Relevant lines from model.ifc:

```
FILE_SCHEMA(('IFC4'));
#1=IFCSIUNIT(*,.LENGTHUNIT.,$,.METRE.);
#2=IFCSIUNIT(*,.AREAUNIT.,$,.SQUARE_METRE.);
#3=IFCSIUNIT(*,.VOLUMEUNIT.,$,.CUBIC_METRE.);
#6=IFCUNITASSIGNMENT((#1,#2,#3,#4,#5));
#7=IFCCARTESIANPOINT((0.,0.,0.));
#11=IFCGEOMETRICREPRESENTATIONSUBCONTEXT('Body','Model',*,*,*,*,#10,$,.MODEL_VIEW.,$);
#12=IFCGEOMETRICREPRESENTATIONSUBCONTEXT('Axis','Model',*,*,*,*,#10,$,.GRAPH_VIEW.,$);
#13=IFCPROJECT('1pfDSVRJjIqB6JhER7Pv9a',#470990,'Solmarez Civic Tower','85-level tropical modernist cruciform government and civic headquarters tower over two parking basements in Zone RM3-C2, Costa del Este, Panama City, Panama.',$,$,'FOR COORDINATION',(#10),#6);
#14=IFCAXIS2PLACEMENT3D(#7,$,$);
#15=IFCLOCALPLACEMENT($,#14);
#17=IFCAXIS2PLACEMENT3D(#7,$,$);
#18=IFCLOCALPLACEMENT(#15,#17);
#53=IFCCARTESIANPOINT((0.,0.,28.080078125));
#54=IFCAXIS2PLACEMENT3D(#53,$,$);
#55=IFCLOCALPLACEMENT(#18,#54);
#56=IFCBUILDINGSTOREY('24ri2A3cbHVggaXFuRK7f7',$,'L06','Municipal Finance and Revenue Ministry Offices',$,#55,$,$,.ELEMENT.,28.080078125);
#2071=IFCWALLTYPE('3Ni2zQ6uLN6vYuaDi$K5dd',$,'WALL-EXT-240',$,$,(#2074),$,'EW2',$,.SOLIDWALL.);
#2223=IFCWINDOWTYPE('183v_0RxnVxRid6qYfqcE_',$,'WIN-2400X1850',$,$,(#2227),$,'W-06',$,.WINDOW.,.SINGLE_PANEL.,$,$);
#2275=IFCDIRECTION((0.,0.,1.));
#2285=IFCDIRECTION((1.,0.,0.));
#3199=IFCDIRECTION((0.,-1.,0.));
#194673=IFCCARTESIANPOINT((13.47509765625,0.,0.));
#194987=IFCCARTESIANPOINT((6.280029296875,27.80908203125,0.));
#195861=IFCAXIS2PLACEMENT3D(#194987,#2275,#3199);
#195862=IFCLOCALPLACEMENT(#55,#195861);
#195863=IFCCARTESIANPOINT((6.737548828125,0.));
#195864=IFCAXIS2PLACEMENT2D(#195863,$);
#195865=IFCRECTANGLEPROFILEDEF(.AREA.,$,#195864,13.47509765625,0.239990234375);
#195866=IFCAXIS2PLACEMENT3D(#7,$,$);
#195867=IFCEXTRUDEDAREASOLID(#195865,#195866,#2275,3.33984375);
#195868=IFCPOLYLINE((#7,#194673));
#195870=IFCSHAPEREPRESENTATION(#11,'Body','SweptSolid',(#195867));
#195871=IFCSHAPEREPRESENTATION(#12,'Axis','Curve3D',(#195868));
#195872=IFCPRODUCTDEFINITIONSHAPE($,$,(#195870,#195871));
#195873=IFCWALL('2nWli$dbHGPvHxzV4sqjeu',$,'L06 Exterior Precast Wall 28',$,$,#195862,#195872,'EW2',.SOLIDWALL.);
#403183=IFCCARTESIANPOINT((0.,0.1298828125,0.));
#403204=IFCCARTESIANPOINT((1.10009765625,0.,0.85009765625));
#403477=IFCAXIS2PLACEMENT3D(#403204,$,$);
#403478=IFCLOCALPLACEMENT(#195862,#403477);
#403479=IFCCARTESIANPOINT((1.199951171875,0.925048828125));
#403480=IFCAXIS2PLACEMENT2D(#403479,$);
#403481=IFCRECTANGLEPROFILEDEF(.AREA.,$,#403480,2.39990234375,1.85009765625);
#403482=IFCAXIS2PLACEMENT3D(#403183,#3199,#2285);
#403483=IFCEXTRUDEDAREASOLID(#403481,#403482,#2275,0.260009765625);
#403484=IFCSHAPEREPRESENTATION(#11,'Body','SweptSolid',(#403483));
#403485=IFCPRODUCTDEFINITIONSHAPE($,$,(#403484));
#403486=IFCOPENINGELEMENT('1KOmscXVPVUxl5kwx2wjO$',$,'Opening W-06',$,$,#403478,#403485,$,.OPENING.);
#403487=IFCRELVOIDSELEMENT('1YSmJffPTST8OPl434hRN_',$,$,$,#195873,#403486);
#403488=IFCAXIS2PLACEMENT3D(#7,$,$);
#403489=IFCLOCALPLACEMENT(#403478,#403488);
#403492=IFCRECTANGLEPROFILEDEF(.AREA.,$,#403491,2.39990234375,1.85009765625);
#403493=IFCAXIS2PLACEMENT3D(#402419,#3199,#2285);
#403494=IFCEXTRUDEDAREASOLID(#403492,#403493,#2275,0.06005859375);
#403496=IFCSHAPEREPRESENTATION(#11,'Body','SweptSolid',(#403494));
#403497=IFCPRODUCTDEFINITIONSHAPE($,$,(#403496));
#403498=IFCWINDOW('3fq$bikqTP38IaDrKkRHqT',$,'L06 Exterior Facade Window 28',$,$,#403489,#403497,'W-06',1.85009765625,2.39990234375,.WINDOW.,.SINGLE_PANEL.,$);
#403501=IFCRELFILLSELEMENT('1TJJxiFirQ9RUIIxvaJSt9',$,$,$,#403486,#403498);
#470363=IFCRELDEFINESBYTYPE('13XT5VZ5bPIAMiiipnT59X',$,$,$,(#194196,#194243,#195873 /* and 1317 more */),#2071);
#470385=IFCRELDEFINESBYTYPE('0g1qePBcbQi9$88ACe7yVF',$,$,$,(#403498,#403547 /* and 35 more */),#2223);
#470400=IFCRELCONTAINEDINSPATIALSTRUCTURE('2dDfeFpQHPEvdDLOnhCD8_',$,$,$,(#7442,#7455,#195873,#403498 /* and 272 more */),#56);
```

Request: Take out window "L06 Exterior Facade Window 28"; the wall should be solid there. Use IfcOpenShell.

```python
import ifcopenshell
import ifcopenshell.api.feature
import ifcopenshell.api.root
import ifcopenshell.geom
import ifcopenshell.util.shape

model = ifcopenshell.open("model.ifc")
settings = ifcopenshell.geom.settings()


def volume(element):
    """Net volume in cubic metres, openings subtracted."""
    shape = ifcopenshell.geom.create_shape(settings, element)
    return ifcopenshell.util.shape.get_volume(shape.geometry)


window = model.by_guid("3fq$bikqTP38IaDrKkRHqT")
opening = window.FillsVoids[0].RelatingOpeningElement
wall = opening.VoidsElements[0].RelatingBuildingElement
before = volume(wall)

ifcopenshell.api.root.remove_product(model, product=window)
ifcopenshell.api.feature.remove_feature(model, feature=opening)

after = volume(wall)

print(f"wall volume {before:.3f} -> {after:.3f} m3")

model.write("model_rev.ifc")
```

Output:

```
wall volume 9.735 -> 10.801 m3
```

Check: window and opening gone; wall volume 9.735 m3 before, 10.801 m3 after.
